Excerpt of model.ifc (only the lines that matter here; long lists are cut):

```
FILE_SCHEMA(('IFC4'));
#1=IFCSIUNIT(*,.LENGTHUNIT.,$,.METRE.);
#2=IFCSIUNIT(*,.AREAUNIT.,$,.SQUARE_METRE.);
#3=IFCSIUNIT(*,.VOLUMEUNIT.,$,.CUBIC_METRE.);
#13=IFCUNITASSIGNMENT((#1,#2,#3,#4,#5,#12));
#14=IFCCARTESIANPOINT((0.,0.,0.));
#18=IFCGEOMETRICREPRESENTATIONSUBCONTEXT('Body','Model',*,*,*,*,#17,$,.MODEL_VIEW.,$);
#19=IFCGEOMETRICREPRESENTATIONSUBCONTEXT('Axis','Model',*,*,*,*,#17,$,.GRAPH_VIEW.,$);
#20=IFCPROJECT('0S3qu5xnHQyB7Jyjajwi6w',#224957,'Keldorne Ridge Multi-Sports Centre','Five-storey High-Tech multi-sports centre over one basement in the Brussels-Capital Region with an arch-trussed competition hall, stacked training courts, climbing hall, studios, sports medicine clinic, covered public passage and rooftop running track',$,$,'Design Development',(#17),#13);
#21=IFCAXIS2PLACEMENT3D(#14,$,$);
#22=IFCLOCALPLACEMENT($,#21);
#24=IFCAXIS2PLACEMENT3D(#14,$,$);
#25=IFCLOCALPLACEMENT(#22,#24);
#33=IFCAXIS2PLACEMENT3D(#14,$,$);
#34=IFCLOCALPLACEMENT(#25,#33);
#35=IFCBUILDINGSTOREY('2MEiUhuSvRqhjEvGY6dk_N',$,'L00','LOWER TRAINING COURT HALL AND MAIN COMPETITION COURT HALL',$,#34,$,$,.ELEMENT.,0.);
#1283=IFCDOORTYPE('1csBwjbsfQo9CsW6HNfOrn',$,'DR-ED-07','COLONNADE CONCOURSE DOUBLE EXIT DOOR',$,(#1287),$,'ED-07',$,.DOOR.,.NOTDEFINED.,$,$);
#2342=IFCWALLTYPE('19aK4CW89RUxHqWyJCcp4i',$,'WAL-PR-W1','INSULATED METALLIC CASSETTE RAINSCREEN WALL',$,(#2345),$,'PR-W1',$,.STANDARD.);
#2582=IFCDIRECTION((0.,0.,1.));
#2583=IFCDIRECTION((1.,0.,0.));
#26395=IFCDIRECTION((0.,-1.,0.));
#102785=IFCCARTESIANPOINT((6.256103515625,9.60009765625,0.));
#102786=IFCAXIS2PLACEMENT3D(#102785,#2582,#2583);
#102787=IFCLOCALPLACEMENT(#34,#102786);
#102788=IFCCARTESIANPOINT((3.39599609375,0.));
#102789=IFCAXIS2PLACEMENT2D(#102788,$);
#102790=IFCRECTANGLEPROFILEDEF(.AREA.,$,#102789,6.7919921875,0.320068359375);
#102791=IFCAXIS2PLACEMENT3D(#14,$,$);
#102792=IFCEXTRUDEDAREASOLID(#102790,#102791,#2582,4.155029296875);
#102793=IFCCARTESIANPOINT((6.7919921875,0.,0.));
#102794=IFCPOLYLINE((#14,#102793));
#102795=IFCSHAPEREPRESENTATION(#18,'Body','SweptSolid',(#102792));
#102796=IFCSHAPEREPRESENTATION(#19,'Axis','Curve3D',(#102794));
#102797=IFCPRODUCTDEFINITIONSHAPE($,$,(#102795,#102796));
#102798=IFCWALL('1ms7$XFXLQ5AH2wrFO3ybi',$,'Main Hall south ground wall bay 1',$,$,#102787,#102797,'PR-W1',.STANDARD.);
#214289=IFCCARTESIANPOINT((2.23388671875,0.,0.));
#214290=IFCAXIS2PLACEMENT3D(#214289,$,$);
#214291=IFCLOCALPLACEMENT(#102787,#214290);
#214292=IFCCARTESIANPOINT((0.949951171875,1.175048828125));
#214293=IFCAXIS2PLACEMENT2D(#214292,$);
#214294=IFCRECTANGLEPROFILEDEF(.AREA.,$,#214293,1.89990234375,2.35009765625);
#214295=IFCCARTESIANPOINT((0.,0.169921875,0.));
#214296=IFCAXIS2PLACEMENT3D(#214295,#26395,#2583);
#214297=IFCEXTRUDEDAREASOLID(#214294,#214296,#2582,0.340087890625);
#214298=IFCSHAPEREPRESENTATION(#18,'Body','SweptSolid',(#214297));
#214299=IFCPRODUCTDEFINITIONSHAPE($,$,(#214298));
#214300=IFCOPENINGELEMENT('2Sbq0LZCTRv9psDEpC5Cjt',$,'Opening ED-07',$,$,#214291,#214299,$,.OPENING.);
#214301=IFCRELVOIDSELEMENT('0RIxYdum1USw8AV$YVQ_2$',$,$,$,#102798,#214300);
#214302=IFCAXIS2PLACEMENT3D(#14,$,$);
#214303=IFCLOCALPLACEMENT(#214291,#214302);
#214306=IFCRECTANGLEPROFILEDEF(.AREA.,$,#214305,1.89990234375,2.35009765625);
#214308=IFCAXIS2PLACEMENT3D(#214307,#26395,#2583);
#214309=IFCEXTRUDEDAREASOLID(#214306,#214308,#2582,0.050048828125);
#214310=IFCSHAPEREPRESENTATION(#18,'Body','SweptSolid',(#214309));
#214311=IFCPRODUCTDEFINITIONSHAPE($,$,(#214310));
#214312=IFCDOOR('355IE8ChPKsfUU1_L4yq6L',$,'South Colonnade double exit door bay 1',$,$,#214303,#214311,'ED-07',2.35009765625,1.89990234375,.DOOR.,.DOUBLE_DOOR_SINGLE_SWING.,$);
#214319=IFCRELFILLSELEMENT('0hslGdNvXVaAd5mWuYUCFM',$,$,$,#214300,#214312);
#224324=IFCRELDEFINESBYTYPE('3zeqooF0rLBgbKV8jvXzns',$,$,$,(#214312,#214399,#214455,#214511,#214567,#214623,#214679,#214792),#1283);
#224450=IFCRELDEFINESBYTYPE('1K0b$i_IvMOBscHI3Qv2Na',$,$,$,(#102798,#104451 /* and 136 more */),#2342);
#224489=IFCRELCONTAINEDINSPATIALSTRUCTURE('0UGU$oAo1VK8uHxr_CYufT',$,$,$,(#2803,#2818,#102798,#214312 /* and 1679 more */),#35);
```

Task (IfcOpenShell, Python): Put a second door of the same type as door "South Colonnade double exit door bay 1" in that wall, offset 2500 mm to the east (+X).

```python
import ifcopenshell
import ifcopenshell.api.feature
import ifcopenshell.api.geometry
import ifcopenshell.api.root
import ifcopenshell.geom
import ifcopenshell.util.element
import ifcopenshell.util.placement
import ifcopenshell.util.shape

model = ifcopenshell.open("model.ifc")
settings = ifcopenshell.geom.settings()


def volume(element):
    """Net volume in cubic metres, openings subtracted."""
    shape = ifcopenshell.geom.create_shape(settings, element)
    return ifcopenshell.util.shape.get_volume(shape.geometry)


door = model.by_id(214312)
opening = door.FillsVoids[0].RelatingOpeningElement
wall = opening.VoidsElements[0].RelatingBuildingElement
before = volume(wall)
shift = ifcopenshell.util.placement.get_local_placement(wall.ObjectPlacement)[:3, 0] * 2.5

# copy_class copies the void relationship, type, container and properties, but no geometry.
new_opening = ifcopenshell.api.root.copy_class(model, product=opening)
new_opening.Representation = ifcopenshell.util.element.copy_deep(
    model, opening.Representation, exclude=["IfcGeometricRepresentationContext", "IfcRepresentationMap"]
)
new_door = ifcopenshell.api.root.copy_class(model, product=door)
new_door.Representation = ifcopenshell.util.element.copy_deep(
    model, door.Representation, exclude=["IfcGeometricRepresentationContext", "IfcRepresentationMap"]
)
new_door.Tag = None
ifcopenshell.api.feature.add_filling(model, opening=new_opening, element=new_door)

for old, new in ((opening, new_opening), (door, new_door)):
    matrix = ifcopenshell.util.placement.get_local_placement(old.ObjectPlacement)
    matrix[:3, 3] += shift
    ifcopenshell.api.geometry.edit_object_placement(model, product=new, matrix=matrix, is_si=False)

after = volume(wall)

print(f"wall volume {before:.3f} -> {after:.3f} m3")

model.write("model_edited.ifc")
```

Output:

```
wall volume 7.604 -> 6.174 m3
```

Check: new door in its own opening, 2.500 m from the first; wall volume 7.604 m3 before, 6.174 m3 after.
